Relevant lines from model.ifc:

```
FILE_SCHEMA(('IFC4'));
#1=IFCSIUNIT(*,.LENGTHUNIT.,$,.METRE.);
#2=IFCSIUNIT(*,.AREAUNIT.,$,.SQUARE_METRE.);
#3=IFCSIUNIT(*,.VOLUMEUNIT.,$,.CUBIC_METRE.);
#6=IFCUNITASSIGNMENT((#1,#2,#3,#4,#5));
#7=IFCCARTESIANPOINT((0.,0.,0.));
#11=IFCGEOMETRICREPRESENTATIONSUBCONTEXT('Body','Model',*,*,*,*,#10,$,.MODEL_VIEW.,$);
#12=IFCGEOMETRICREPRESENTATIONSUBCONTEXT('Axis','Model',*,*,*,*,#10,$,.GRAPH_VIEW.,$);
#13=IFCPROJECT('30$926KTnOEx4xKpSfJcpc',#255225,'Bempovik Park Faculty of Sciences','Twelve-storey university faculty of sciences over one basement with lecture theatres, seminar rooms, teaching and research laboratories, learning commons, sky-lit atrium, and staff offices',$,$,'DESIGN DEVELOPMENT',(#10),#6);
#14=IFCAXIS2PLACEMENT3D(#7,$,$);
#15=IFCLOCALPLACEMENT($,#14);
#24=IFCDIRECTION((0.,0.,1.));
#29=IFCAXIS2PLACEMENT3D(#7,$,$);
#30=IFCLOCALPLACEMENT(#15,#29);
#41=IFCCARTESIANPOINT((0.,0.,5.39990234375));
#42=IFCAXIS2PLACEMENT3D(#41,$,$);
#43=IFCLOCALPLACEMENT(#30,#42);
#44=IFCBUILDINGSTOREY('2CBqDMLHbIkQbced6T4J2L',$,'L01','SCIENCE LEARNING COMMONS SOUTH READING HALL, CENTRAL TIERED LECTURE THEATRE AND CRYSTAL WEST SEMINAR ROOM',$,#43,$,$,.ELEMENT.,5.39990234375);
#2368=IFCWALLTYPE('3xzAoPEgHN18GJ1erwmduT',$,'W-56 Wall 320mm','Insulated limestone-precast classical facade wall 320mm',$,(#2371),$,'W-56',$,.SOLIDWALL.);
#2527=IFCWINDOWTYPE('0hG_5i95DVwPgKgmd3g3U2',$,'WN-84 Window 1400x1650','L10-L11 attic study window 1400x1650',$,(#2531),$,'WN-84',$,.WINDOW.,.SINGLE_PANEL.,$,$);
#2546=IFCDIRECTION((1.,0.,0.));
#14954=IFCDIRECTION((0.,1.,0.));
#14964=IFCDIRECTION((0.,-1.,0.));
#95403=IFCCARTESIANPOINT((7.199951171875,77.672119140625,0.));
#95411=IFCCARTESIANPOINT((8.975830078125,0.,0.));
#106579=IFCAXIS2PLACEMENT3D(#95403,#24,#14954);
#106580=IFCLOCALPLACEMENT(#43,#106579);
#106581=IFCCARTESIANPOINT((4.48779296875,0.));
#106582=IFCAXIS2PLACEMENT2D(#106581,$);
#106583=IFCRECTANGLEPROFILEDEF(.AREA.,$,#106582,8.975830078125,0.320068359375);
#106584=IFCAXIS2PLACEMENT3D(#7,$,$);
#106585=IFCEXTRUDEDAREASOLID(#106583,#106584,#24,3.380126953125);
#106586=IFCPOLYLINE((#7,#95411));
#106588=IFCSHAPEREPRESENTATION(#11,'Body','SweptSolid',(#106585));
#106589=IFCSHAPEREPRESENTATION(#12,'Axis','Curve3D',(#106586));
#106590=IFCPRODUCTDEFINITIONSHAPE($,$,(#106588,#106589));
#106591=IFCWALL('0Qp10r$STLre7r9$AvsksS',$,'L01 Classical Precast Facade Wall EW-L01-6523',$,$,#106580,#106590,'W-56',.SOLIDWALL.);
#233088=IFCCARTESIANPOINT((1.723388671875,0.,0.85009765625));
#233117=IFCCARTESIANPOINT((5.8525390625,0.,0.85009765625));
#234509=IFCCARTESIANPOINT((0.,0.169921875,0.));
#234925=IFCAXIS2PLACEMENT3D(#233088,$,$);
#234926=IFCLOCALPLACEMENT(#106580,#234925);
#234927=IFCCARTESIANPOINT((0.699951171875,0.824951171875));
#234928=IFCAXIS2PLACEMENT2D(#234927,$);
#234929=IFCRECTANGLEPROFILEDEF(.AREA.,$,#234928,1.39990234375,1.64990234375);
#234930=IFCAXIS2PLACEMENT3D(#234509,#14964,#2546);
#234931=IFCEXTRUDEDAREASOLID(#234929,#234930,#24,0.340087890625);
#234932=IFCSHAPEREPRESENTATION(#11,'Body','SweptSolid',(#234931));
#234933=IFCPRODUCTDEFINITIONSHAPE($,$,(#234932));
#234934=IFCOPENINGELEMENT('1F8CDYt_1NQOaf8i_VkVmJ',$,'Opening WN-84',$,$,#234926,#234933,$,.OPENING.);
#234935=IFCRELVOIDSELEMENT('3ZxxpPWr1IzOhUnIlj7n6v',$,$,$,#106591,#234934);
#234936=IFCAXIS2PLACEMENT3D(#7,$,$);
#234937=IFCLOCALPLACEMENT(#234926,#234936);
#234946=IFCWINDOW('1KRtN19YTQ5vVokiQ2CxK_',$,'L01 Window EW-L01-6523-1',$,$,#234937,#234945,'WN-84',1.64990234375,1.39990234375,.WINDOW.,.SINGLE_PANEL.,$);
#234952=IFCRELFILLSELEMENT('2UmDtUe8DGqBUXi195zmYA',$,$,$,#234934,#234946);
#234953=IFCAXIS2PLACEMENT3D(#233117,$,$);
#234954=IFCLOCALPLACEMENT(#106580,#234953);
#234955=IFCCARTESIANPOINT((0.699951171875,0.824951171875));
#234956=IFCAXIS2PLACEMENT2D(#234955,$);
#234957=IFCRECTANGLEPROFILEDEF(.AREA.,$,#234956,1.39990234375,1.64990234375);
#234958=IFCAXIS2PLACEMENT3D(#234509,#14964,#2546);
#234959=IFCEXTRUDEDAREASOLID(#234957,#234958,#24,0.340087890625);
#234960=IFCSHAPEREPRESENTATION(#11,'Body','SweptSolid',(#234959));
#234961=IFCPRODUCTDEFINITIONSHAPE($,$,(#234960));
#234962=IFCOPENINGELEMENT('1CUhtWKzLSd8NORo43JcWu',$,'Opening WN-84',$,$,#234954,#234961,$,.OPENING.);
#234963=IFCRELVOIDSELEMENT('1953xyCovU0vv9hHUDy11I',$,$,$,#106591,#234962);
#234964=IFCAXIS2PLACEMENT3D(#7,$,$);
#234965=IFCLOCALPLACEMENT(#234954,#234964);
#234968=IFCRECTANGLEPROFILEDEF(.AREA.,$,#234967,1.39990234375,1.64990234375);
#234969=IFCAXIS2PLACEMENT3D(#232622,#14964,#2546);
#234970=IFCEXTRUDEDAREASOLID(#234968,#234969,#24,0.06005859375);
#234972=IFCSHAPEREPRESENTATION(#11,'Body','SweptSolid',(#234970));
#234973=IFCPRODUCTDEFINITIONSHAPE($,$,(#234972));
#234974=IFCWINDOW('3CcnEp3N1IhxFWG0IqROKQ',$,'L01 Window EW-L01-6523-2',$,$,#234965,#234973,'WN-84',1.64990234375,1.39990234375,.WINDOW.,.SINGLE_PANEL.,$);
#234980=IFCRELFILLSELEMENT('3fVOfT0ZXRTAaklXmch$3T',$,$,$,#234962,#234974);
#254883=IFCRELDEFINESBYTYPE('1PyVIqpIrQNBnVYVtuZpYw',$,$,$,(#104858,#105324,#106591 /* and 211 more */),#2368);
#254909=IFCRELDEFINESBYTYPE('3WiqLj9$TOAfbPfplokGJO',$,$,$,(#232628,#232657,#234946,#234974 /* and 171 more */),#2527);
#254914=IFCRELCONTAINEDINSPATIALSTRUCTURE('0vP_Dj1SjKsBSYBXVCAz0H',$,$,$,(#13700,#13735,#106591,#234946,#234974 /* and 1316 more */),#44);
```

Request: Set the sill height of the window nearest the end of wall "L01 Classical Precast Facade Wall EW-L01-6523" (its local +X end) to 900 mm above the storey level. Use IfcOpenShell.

```python
import numpy as np
import ifcopenshell
import ifcopenshell.api.geometry
import ifcopenshell.geom
import ifcopenshell.util.element
import ifcopenshell.util.placement
import ifcopenshell.util.shape
import ifcopenshell.util.unit

model = ifcopenshell.open("model.ifc")
unit_scale = ifcopenshell.util.unit.calculate_unit_scale(model)

window = model.by_guid("3CcnEp3N1IhxFWG0IqROKQ")
opening = window.FillsVoids[0].RelatingOpeningElement
storey = ifcopenshell.util.element.get_container(window, ifc_class="IfcBuildingStorey")
level = ifcopenshell.util.placement.get_local_placement(storey.ObjectPlacement)[2, 3]

# The opening's origin need not be at the sill, so measure its lowest point.
shape = ifcopenshell.geom.create_shape(ifcopenshell.geom.settings(), opening)
bottom = ifcopenshell.util.shape.get_shape_bottom_elevation(shape, shape.geometry) / unit_scale
dz = level + 0.9 - bottom

shift = np.array([0.0, 0.0, dz])
# The window is placed relative to its opening, so it follows when the opening moves.
matrix = ifcopenshell.util.placement.get_local_placement(opening.ObjectPlacement)
matrix[:3, 3] += shift
ifcopenshell.api.geometry.edit_object_placement(
    model, product=opening, matrix=matrix, is_si=False, should_transform_children=True
)

print(f"moved by {dz * unit_scale:+.3f} m")

model.write("model_v2.ifc")
```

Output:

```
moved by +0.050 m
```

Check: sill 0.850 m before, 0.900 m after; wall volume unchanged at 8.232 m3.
